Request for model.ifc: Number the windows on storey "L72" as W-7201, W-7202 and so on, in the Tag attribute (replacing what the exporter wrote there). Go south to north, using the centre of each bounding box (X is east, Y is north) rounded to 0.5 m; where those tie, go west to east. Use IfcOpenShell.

First a look at what the model holds.

```python
import ifcopenshell
import ifcopenshell.util.element
import ifcopenshell.util.placement

model = ifcopenshell.open("model.ifc")
print(model.schema)
storey = next(s for s in model.by_type("IfcBuildingStorey") if s.Name == "L72")
windows = [e for e in ifcopenshell.util.element.get_decomposition(storey) if e.is_a("IfcWindow")]
for e in sorted(windows, key=lambda e: e.id()):
    origin = ifcopenshell.util.placement.get_local_placement(e.ObjectPlacement)[:3, 3]
    print(e.id(), e.Tag, e.Name, origin.round(2) + 0.0, sep=" | ")
```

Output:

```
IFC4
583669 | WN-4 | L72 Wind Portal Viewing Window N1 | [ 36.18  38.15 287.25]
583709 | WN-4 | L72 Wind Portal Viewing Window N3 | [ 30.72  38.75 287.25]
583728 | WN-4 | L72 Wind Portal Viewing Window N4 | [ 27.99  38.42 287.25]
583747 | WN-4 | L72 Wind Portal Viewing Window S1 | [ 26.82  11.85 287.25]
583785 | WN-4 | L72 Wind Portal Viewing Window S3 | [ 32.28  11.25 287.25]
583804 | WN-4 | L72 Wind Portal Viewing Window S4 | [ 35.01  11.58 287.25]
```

```python
import ifcopenshell
import ifcopenshell.geom
import ifcopenshell.util.element
import ifcopenshell.util.shape

model = ifcopenshell.open("model.ifc")
settings = ifcopenshell.geom.settings()
settings.set("use-world-coords", True)


def centre(element):
    shape = ifcopenshell.geom.create_shape(settings, element)
    return ifcopenshell.util.shape.get_bbox_centroid(shape.geometry)


storey = next(s for s in model.by_type("IfcBuildingStorey") if s.Name == "L72")
windows = [e for e in ifcopenshell.util.element.get_decomposition(storey) if e.is_a("IfcWindow")]

# Insertion points can sit at a corner or the storey origin, so sort by the geometry (in metres).
centres = {e: centre(e) for e in windows}
windows.sort(key=lambda e: (round(centres[e][1] / 0.5), centres[e][0]))

for i, e in enumerate(windows, start=1):
    number = f"W-72{i:02d}"
    e.Tag = number
    print(e.id(), number)

model.write("model_v2.ifc")
```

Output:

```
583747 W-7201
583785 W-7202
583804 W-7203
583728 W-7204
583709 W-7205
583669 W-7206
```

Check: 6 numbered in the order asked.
